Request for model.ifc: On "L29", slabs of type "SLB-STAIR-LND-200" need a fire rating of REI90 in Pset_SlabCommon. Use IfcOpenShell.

First a look at what the model holds.

```python
import ifcopenshell
import ifcopenshell.util.element

model = ifcopenshell.open("model.ifc")
print(model.schema)
storey = next(s for s in model.by_type("IfcBuildingStorey") if s.Name == "L29")
slabs = [e for e in ifcopenshell.util.element.get_decomposition(storey) if e.is_a("IfcSlab")]
seen = {}
for e in slabs:
    element_type = ifcopenshell.util.element.get_type(e)
    key = (element_type.Name if element_type != e and element_type else None, ifcopenshell.util.element.get_pset(e, "Pset_SlabCommon", "FireRating"))
    seen[key] = seen.get(key, 0) + 1
for (name, value), count in sorted(seen.items(), key=str):
    print(count, "x", name, "|", value)
```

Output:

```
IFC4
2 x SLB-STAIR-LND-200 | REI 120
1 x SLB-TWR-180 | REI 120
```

```python
import ifcopenshell
import ifcopenshell.api.pset
import ifcopenshell.util.element

model = ifcopenshell.open("model.ifc")

storey = next(s for s in model.by_type("IfcBuildingStorey") if s.Name == "L29")
slabs = [e for e in ifcopenshell.util.element.get_decomposition(storey) if e.is_a("IfcSlab")]

count = 0
for e in slabs:
    element_type = ifcopenshell.util.element.get_type(e)
    if element_type in (None, e) or element_type.Name != "SLB-STAIR-LND-200":
        continue
    found = ifcopenshell.util.element.get_pset(e, "Pset_SlabCommon", should_inherit=False)
    if found:
        pset = model.by_id(found["id"])
        if len(ifcopenshell.util.element.get_elements_by_pset(pset)) > 1:
            pset = ifcopenshell.api.pset.unshare_pset(model, products=[e], pset=pset)[0]
    else:
        pset = ifcopenshell.api.pset.add_pset(model, product=e, name="Pset_SlabCommon")
    ifcopenshell.api.pset.edit_pset(model, pset=pset, properties={"FireRating": "REI90"})
    count += 1

print(count, "slabs updated")

model.write("model_updated.ifc")
```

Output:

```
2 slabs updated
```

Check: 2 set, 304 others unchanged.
